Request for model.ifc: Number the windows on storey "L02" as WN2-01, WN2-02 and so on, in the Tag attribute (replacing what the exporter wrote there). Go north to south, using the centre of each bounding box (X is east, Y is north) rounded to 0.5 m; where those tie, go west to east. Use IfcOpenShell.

First a look at what the model holds.

```python
import ifcopenshell
import ifcopenshell.util.element
import ifcopenshell.util.placement

model = ifcopenshell.open("model.ifc")
print(model.schema)
storey = next(s for s in model.by_type("IfcBuildingStorey") if s.Name == "L02")
windows = [e for e in ifcopenshell.util.element.get_decomposition(storey) if e.is_a("IfcWindow")]
for e in sorted(windows, key=lambda e: e.id()):
    origin = ifcopenshell.util.placement.get_local_placement(e.ObjectPlacement)[:3, 3]
    print(e.id(), e.Tag, e.Name, origin.round(2) + 0.0, sep=" | ")
```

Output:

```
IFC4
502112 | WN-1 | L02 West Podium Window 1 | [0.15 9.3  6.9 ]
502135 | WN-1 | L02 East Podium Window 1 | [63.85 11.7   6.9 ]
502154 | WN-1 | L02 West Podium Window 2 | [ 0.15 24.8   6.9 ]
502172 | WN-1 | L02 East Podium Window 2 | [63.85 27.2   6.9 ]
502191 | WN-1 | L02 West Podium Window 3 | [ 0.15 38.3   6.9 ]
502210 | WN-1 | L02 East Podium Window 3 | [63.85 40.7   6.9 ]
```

```python
import ifcopenshell
import ifcopenshell.geom
import ifcopenshell.util.element
import ifcopenshell.util.shape

model = ifcopenshell.open("model.ifc")
settings = ifcopenshell.geom.settings()
settings.set("use-world-coords", True)


def centre(element):
    shape = ifcopenshell.geom.create_shape(settings, element)
    return ifcopenshell.util.shape.get_bbox_centroid(shape.geometry)


storey = next(s for s in model.by_type("IfcBuildingStorey") if s.Name == "L02")
windows = [e for e in ifcopenshell.util.element.get_decomposition(storey) if e.is_a("IfcWindow")]

# Insertion points can sit at a corner or the storey origin, so sort by the geometry (in metres).
centres = {e: centre(e) for e in windows}
windows.sort(key=lambda e: (-round(centres[e][1] / 0.5), centres[e][0]))

for i, e in enumerate(windows, start=1):
    number = f"WN2-{i:02d}"
    e.Tag = number
    print(e.id(), number)

model.write("model_v2.ifc")
```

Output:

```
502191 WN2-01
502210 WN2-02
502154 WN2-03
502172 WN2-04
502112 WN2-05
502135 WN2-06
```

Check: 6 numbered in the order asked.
